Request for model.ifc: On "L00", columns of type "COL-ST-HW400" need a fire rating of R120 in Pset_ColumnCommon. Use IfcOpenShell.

First a look at what the model holds.

```python
import ifcopenshell
import ifcopenshell.util.element

model = ifcopenshell.open("model.ifc")
print(model.schema)
storey = next(s for s in model.by_type("IfcBuildingStorey") if s.Name == "L00")
columns = [e for e in ifcopenshell.util.element.get_decomposition(storey) if e.is_a("IfcColumn")]
seen = {}
for e in columns:
    element_type = ifcopenshell.util.element.get_type(e)
    key = (element_type.Name if element_type != e and element_type else None, ifcopenshell.util.element.get_pset(e, "Pset_ColumnCommon", "FireRating"))
    seen[key] = seen.get(key, 0) + 1
for (name, value), count in sorted(seen.items(), key=str):
    print(count, "x", name, "|", value)
```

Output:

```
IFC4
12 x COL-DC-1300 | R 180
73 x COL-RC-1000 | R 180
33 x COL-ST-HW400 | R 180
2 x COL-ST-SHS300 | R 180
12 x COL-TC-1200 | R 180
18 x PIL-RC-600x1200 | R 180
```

```python
import ifcopenshell
import ifcopenshell.api.pset
import ifcopenshell.util.element

model = ifcopenshell.open("model.ifc")

storey = next(s for s in model.by_type("IfcBuildingStorey") if s.Name == "L00")
columns = [e for e in ifcopenshell.util.element.get_decomposition(storey) if e.is_a("IfcColumn")]

count = 0
for e in columns:
    element_type = ifcopenshell.util.element.get_type(e)
    if element_type in (None, e) or element_type.Name != "COL-ST-HW400":
        continue
    # add_pset returns the element's existing set when there is one.
    pset = ifcopenshell.api.pset.add_pset(model, product=e, name="Pset_ColumnCommon")
    ifcopenshell.api.pset.edit_pset(model, pset=pset, properties={"FireRating": "R120"})
    count += 1

print(count, "columns updated")

model.write("model-out.ifc")
```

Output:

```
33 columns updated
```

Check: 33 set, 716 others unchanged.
